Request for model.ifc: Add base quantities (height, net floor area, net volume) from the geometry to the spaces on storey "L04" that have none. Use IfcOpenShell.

First a look at what the model holds.

```python
import ifcopenshell
import ifcopenshell.util.element
import ifcopenshell.util.unit

model = ifcopenshell.open("model.ifc")
print(model.schema)
for unit_type in ("LENGTHUNIT", "AREAUNIT", "VOLUMEUNIT"):
    print(unit_type, ifcopenshell.util.unit.calculate_unit_scale(model, unit_type))
storey = next(s for s in model.by_type("IfcBuildingStorey") if s.Name == "L04")
spaces = [e for e in ifcopenshell.util.element.get_decomposition(storey) if e.is_a("IfcSpace")]
for e in sorted(spaces, key=lambda e: e.id()):
    print(e.id(), e.is_a(), e.Name, list(ifcopenshell.util.element.get_psets(e, qtos_only=True)), sep=" | ")
```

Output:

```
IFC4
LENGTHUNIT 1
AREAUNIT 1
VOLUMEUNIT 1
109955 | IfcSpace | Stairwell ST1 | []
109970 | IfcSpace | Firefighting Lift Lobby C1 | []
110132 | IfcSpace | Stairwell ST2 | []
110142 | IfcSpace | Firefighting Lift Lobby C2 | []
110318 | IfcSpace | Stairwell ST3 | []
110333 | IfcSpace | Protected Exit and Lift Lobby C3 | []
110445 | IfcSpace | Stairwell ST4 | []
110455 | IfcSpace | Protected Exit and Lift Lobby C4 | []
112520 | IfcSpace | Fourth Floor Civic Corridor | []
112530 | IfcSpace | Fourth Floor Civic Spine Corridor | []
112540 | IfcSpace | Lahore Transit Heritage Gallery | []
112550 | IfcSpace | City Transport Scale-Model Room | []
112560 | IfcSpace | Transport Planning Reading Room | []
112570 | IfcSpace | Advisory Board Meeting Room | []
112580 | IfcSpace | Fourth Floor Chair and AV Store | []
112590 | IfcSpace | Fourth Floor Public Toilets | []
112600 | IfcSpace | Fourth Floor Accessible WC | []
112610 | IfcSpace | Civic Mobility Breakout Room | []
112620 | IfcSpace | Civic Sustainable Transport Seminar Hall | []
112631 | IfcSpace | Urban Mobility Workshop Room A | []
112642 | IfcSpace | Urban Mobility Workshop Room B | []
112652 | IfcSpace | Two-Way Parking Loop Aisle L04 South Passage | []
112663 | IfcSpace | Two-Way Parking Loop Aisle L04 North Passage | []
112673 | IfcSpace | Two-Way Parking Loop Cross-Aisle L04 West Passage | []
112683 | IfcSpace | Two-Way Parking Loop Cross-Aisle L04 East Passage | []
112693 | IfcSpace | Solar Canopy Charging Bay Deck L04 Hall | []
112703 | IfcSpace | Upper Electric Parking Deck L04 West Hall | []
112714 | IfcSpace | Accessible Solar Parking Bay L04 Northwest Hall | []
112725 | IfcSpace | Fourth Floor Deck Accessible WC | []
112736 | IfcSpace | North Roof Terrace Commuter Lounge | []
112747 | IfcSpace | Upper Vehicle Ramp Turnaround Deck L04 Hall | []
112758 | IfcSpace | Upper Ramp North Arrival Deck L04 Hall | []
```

```python
import ifcopenshell
import ifcopenshell.api.pset
import ifcopenshell.geom
import ifcopenshell.util.element
import ifcopenshell.util.shape
import ifcopenshell.util.unit

model = ifcopenshell.open("model.ifc")
unit_scale = ifcopenshell.util.unit.calculate_unit_scale(model)
area_scale = ifcopenshell.util.unit.calculate_unit_scale(model, "AREAUNIT")
volume_scale = ifcopenshell.util.unit.calculate_unit_scale(model, "VOLUMEUNIT")
settings = ifcopenshell.geom.settings()

storey = next(s for s in model.by_type("IfcBuildingStorey") if s.Name == "L04")
spaces = [e for e in ifcopenshell.util.element.get_decomposition(storey) if e.is_a("IfcSpace")]

for e in sorted(spaces, key=lambda e: e.id()):
    if ifcopenshell.util.element.get_psets(e, qtos_only=True, should_inherit=False):
        continue
    # Geometry comes back in metres, in the element's own axes.
    shape = ifcopenshell.geom.create_shape(settings, e)
    values = {
        "Height": ifcopenshell.util.shape.get_z(shape.geometry) / unit_scale,
        "NetFloorArea": ifcopenshell.util.shape.get_footprint_area(shape.geometry) / area_scale,
        "NetVolume": ifcopenshell.util.shape.get_volume(shape.geometry) / volume_scale,
    }
    qto = ifcopenshell.api.pset.add_qto(model, product=e, name="Qto_SpaceBaseQuantities")
    ifcopenshell.api.pset.edit_qto(model, qto=qto, properties=values)
    print(e.id(), {k: round(v, 3) for k, v in values.items()})

model.write("model_edited.ifc")
```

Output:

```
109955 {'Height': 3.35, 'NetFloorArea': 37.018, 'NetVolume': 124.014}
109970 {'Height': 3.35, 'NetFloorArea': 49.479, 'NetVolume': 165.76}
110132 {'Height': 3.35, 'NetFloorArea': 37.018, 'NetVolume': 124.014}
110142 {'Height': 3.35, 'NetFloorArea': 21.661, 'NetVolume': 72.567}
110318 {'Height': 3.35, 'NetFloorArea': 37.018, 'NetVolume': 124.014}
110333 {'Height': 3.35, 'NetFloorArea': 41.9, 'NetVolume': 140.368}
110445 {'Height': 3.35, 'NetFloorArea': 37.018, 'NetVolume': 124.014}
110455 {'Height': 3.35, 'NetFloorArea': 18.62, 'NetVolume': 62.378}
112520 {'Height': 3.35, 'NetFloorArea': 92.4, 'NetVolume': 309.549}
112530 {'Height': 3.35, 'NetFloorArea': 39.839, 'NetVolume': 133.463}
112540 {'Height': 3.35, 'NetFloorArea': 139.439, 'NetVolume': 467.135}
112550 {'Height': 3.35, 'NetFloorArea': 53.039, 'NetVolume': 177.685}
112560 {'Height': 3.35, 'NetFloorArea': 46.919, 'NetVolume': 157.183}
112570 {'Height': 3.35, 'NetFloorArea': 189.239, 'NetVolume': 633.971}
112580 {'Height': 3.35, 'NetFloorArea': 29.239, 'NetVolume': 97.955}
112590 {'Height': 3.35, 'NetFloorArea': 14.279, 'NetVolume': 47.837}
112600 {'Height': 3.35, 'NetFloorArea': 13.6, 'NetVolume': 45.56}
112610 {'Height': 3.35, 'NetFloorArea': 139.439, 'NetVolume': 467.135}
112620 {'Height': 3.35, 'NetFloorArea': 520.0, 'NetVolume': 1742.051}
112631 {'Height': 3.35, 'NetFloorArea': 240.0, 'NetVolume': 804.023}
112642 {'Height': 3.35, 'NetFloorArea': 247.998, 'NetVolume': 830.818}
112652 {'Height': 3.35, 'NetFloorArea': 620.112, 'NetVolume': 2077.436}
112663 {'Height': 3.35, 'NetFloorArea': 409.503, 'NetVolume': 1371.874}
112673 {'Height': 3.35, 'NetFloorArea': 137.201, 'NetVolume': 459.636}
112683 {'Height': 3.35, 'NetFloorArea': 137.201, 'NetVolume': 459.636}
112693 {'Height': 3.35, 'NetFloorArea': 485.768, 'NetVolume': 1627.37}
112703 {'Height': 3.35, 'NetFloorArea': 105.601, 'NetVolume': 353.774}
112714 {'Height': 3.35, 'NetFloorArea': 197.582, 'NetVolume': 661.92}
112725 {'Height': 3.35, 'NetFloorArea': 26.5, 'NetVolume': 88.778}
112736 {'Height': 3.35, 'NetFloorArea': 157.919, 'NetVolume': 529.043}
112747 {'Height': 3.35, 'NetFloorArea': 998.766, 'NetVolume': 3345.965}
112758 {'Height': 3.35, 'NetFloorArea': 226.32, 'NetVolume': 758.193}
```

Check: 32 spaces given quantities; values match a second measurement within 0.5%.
